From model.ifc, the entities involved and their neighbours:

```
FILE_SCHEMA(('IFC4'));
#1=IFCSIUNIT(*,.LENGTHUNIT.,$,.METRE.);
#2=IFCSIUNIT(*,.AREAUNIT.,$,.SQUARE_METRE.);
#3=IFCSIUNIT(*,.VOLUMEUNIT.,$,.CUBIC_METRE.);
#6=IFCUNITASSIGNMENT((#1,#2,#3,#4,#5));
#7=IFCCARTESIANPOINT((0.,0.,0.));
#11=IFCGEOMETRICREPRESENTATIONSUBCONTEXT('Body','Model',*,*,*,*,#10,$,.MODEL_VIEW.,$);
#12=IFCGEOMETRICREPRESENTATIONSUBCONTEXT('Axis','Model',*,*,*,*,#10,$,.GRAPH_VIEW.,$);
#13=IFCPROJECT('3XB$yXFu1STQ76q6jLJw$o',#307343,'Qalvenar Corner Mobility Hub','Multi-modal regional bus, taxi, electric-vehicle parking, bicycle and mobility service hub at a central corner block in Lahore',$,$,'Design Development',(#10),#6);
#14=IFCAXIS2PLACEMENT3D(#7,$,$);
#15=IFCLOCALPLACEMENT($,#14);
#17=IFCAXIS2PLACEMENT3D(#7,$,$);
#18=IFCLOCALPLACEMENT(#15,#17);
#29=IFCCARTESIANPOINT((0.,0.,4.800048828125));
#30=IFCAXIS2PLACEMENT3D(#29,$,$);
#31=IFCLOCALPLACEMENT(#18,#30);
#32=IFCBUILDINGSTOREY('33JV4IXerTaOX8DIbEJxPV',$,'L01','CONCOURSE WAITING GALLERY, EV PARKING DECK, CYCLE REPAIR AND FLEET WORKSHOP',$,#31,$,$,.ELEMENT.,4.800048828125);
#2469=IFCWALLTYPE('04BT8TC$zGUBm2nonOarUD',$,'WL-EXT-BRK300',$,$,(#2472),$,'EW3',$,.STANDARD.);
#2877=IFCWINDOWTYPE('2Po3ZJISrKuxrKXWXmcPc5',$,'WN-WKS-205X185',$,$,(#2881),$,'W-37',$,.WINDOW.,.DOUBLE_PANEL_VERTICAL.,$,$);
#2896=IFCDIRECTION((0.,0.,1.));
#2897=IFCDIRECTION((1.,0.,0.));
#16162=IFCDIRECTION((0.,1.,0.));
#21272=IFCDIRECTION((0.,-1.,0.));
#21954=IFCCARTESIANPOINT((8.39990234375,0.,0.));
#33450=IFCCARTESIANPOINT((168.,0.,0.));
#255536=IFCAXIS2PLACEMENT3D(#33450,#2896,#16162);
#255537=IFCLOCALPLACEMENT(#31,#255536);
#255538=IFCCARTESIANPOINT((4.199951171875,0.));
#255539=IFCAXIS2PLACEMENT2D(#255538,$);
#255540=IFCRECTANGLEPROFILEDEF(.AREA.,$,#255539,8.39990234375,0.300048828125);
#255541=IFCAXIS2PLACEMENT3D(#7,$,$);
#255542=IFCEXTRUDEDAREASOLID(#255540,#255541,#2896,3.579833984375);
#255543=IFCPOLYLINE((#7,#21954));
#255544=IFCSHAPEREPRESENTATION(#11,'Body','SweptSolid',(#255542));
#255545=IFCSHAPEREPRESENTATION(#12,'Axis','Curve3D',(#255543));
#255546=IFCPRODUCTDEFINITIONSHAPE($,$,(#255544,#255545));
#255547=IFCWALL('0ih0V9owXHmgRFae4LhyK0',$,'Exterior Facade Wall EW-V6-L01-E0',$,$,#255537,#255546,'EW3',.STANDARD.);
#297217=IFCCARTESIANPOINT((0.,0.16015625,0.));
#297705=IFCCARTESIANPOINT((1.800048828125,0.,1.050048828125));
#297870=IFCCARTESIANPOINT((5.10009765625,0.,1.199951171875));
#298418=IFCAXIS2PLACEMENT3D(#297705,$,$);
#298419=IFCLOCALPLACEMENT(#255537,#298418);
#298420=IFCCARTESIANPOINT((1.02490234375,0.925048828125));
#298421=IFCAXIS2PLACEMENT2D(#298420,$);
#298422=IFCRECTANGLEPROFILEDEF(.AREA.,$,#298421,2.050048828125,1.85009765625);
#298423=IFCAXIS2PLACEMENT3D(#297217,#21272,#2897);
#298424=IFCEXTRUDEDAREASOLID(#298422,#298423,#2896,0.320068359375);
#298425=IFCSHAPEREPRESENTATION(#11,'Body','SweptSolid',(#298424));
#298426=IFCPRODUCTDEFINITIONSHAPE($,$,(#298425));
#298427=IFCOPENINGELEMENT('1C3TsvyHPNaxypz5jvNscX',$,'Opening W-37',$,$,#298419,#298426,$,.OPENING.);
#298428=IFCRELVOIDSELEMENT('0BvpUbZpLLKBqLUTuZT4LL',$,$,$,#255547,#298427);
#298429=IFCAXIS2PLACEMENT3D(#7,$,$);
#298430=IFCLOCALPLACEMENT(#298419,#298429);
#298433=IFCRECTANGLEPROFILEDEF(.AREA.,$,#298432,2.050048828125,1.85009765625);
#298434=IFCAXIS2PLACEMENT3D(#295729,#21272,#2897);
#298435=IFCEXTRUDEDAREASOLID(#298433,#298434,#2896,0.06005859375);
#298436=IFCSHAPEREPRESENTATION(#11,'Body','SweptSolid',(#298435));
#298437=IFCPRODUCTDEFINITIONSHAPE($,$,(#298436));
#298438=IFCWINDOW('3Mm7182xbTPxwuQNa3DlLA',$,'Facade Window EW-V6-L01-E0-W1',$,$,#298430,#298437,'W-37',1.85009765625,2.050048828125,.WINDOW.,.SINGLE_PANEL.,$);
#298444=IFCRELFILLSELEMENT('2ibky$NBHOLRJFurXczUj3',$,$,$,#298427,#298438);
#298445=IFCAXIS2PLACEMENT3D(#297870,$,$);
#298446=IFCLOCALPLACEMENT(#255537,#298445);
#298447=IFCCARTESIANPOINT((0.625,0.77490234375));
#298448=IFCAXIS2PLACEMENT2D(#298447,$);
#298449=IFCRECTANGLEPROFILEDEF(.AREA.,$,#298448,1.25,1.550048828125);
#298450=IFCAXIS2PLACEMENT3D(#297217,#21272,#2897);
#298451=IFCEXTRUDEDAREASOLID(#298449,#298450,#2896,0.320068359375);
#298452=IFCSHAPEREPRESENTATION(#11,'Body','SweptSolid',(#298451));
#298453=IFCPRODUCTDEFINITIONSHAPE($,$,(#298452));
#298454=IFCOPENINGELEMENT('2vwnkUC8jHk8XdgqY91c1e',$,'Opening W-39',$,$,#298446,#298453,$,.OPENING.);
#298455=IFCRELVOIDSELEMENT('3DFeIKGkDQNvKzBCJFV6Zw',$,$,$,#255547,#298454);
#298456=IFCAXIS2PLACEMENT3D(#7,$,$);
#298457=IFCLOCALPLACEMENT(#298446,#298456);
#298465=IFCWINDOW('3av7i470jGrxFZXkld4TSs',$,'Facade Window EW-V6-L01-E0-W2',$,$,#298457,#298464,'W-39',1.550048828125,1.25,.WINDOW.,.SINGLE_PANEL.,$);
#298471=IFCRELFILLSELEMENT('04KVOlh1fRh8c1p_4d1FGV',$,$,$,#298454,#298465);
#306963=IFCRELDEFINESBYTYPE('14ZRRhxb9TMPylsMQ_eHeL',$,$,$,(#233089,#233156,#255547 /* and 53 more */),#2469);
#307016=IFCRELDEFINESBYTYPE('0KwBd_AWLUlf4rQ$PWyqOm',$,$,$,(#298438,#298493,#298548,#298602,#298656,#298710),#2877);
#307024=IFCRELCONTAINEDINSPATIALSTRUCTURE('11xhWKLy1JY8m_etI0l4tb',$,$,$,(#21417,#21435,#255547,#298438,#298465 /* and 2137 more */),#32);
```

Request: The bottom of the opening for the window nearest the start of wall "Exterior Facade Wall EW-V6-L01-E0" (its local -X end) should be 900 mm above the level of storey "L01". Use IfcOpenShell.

```python
import numpy as np
import ifcopenshell
import ifcopenshell.api.geometry
import ifcopenshell.geom
import ifcopenshell.util.element
import ifcopenshell.util.placement
import ifcopenshell.util.shape
import ifcopenshell.util.unit

model = ifcopenshell.open("model.ifc")
unit_scale = ifcopenshell.util.unit.calculate_unit_scale(model)

window = model.by_id(298438)
opening = window.FillsVoids[0].RelatingOpeningElement
storey = ifcopenshell.util.element.get_container(window, ifc_class="IfcBuildingStorey")
level = ifcopenshell.util.placement.get_local_placement(storey.ObjectPlacement)[2, 3]

# The opening's origin need not be at the sill, so measure its lowest point.
shape = ifcopenshell.geom.create_shape(ifcopenshell.geom.settings(), opening)
bottom = ifcopenshell.util.shape.get_shape_bottom_elevation(shape, shape.geometry) / unit_scale
dz = level + 0.9 - bottom

shift = np.array([0.0, 0.0, dz])
# The window is placed relative to its opening, so it follows when the opening moves.
matrix = ifcopenshell.util.placement.get_local_placement(opening.ObjectPlacement)
matrix[:3, 3] += shift
ifcopenshell.api.geometry.edit_object_placement(
    model, product=opening, matrix=matrix, is_si=False, should_transform_children=True
)

print(f"moved by {dz * unit_scale:+.3f} m")

model.write("model_edited.ifc")
```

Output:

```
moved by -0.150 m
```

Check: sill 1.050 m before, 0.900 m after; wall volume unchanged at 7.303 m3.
